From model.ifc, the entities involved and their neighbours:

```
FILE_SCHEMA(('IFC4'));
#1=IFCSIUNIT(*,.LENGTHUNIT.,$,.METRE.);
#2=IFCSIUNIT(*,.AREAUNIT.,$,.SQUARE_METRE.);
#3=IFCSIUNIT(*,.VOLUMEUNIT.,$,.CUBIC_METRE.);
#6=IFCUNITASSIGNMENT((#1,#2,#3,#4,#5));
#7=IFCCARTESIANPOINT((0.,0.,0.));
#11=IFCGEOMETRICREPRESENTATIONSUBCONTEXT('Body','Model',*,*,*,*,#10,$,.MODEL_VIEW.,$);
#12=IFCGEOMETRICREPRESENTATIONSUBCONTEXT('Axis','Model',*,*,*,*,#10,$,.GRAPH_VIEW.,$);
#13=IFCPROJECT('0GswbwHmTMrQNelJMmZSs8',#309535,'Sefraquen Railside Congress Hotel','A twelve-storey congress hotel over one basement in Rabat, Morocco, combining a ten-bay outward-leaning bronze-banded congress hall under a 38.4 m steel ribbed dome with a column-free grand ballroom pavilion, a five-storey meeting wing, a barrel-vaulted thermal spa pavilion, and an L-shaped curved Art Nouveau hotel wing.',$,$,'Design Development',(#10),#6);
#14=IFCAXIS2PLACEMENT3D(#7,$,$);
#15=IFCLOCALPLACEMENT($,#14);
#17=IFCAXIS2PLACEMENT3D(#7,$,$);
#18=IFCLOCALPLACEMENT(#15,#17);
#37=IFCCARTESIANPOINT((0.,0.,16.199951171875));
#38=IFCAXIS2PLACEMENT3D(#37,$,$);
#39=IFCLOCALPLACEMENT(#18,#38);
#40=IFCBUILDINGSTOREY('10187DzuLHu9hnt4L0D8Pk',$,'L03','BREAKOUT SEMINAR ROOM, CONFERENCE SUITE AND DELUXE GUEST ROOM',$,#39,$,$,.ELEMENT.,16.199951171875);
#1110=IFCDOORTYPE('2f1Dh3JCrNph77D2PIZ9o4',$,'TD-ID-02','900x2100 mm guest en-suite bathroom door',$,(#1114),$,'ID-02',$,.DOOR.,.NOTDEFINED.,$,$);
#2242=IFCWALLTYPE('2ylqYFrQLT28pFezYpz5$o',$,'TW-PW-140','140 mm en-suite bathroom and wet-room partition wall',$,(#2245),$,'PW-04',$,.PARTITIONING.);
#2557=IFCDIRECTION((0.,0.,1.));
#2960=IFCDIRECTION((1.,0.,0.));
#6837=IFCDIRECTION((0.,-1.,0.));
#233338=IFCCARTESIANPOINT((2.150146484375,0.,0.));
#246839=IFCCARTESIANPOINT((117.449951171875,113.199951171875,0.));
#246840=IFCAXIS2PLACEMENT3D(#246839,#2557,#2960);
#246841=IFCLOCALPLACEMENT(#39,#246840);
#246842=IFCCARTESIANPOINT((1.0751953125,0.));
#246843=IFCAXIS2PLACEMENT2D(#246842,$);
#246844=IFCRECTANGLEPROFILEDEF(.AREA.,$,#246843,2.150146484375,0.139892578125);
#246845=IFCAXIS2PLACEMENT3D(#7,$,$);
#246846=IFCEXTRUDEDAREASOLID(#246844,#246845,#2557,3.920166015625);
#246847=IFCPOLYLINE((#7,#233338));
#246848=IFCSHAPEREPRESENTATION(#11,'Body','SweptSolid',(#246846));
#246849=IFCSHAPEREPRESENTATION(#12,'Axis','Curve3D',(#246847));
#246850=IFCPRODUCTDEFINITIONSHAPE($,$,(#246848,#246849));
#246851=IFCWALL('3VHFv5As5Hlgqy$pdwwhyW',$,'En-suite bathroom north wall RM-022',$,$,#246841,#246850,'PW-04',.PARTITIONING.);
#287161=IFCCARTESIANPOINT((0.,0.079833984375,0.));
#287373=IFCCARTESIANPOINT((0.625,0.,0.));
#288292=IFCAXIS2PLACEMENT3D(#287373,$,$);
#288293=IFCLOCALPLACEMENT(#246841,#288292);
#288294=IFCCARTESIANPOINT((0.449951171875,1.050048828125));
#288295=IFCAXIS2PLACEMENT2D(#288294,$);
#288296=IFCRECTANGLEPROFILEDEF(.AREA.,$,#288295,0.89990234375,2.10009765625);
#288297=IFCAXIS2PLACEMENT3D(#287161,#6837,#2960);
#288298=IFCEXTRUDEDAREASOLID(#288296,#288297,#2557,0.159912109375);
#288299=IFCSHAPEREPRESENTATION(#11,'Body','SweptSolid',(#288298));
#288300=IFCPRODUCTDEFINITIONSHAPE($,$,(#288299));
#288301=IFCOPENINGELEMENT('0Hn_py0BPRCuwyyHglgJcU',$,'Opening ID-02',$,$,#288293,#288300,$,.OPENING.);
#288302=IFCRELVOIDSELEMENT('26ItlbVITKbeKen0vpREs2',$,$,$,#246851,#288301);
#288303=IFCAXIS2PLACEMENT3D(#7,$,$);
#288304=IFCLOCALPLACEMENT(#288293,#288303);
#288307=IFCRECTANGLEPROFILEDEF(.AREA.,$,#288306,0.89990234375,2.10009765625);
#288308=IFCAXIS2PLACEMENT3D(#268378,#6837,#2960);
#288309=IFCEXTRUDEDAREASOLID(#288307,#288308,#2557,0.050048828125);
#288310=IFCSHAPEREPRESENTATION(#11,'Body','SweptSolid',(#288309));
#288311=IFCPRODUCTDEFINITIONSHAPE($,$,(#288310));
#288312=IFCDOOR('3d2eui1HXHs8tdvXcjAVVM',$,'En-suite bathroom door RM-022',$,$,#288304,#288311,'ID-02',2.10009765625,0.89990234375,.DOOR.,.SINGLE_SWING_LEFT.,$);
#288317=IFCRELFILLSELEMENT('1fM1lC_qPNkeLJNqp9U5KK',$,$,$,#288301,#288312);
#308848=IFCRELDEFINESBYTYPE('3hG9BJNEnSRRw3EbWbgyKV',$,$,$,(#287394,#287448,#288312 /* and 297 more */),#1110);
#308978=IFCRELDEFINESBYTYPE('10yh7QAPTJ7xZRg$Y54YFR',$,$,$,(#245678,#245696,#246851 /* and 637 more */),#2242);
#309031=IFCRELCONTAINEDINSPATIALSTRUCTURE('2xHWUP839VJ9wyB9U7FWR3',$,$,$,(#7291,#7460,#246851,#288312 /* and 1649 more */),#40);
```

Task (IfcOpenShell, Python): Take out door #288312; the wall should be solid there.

```python
import ifcopenshell
import ifcopenshell.api.feature
import ifcopenshell.api.root
import ifcopenshell.geom
import ifcopenshell.util.shape

model = ifcopenshell.open("model.ifc")
settings = ifcopenshell.geom.settings()


def volume(element):
    """Net volume in cubic metres, openings subtracted."""
    shape = ifcopenshell.geom.create_shape(settings, element)
    return ifcopenshell.util.shape.get_volume(shape.geometry)


door = model.by_guid("3d2eui1HXHs8tdvXcjAVVM")
opening = door.FillsVoids[0].RelatingOpeningElement
wall = opening.VoidsElements[0].RelatingBuildingElement
before = volume(wall)

ifcopenshell.api.root.remove_product(model, product=door)
ifcopenshell.api.feature.remove_feature(model, feature=opening)

after = volume(wall)

print(f"wall volume {before:.3f} -> {after:.3f} m3")

model.write("model_updated.ifc")
```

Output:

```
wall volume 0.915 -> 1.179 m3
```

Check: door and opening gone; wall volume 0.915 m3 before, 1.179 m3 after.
